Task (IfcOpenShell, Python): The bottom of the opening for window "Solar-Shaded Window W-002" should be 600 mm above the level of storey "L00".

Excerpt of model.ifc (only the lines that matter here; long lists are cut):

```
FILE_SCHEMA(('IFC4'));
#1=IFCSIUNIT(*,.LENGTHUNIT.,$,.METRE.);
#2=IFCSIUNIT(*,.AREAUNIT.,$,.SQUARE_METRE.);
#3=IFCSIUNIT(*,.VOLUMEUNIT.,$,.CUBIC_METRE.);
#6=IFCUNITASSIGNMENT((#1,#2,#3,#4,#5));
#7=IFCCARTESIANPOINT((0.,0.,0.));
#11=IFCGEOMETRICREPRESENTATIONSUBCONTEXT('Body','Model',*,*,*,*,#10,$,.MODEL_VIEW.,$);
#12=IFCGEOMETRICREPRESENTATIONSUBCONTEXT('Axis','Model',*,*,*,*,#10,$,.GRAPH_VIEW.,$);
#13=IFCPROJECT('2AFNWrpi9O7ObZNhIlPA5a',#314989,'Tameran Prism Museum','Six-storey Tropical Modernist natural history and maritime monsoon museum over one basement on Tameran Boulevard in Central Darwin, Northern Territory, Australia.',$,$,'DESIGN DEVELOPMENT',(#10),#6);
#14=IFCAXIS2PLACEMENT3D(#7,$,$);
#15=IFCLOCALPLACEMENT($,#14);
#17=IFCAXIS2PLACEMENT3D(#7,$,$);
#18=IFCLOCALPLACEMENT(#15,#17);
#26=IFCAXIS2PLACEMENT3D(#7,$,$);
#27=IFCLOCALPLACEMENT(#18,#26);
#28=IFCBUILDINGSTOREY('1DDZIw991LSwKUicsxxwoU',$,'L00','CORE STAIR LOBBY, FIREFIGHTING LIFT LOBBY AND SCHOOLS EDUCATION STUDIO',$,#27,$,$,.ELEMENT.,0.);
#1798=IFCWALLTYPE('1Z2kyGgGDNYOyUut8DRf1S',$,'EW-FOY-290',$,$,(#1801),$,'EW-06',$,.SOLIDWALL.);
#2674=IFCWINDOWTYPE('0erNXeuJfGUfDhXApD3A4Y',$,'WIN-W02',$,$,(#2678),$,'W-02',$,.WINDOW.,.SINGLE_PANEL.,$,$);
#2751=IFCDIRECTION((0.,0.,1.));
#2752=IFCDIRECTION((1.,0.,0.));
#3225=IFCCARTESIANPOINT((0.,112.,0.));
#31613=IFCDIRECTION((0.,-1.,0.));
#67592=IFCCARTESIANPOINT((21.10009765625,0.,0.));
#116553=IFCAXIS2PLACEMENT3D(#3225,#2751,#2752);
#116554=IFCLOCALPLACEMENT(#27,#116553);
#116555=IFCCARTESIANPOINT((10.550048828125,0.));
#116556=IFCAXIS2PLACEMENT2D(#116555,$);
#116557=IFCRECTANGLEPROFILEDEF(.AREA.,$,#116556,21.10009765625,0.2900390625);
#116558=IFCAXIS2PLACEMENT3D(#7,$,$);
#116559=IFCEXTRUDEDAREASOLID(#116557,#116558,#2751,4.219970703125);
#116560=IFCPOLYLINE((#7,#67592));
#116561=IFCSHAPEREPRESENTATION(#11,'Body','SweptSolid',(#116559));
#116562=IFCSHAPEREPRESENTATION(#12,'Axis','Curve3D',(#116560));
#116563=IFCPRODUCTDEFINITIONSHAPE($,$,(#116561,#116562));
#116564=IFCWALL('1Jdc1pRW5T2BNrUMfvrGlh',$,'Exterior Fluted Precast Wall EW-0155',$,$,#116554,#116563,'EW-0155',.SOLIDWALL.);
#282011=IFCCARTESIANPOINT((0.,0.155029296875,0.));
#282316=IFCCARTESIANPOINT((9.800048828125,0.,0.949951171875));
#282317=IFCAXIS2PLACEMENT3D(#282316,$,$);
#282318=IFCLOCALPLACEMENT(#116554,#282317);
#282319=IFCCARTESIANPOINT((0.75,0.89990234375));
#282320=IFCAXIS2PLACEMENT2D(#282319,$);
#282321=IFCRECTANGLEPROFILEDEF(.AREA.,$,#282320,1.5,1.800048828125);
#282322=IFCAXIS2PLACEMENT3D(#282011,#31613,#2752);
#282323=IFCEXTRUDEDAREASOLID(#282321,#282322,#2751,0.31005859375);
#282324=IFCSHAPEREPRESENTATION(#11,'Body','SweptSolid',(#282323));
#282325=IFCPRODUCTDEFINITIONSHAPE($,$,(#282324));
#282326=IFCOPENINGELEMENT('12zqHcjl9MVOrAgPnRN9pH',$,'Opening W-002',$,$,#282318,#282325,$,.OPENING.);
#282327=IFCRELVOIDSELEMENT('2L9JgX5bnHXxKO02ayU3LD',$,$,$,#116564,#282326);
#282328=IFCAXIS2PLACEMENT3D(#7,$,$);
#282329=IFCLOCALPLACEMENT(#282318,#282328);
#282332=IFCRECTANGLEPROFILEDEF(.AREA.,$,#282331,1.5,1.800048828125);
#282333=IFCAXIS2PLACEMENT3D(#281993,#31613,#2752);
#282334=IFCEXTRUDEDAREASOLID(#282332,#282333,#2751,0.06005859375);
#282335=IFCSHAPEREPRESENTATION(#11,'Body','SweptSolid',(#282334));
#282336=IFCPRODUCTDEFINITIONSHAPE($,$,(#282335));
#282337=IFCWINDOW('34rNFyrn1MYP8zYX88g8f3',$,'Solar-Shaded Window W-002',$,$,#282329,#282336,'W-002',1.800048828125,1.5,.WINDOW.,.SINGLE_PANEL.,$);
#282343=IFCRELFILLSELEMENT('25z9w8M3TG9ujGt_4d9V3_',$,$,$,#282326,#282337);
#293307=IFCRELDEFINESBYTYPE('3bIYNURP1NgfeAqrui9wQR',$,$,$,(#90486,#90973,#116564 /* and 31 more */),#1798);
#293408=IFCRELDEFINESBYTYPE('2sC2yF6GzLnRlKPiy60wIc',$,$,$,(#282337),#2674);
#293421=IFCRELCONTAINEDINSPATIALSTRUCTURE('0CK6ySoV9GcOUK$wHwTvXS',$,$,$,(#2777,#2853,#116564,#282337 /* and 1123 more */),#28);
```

```python
import numpy as np
import ifcopenshell
import ifcopenshell.api.geometry
import ifcopenshell.geom
import ifcopenshell.util.element
import ifcopenshell.util.placement
import ifcopenshell.util.shape
import ifcopenshell.util.unit

model = ifcopenshell.open("model.ifc")
unit_scale = ifcopenshell.util.unit.calculate_unit_scale(model)

window = model.by_guid("34rNFyrn1MYP8zYX88g8f3")
opening = window.FillsVoids[0].RelatingOpeningElement
storey = ifcopenshell.util.element.get_container(window, ifc_class="IfcBuildingStorey")
level = ifcopenshell.util.placement.get_local_placement(storey.ObjectPlacement)[2, 3]

# The opening's origin need not be at the sill, so measure its lowest point.
shape = ifcopenshell.geom.create_shape(ifcopenshell.geom.settings(), opening)
bottom = ifcopenshell.util.shape.get_shape_bottom_elevation(shape, shape.geometry) / unit_scale
dz = level + 0.6 - bottom

shift = np.array([0.0, 0.0, dz])
# The window is placed relative to its opening, so it follows when the opening moves.
matrix = ifcopenshell.util.placement.get_local_placement(opening.ObjectPlacement)
matrix[:3, 3] += shift
ifcopenshell.api.geometry.edit_object_placement(
    model, product=opening, matrix=matrix, is_si=False, should_transform_children=True
)

print(f"moved by {dz * unit_scale:+.3f} m")

model.write("model_updated.ifc")
```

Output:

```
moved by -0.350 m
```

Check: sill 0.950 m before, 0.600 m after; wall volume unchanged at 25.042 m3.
